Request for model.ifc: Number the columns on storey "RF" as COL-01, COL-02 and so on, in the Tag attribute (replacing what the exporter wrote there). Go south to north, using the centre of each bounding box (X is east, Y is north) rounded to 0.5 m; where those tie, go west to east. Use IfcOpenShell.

First a look at what the model holds.

```python
import ifcopenshell
import ifcopenshell.util.element
import ifcopenshell.util.placement

model = ifcopenshell.open("model.ifc")
print(model.schema)
storey = next(s for s in model.by_type("IfcBuildingStorey") if s.Name == "RF")
columns = [e for e in ifcopenshell.util.element.get_decomposition(storey) if e.is_a("IfcColumn")]
for e in sorted(columns, key=lambda e: e.id()):
    origin = ifcopenshell.util.placement.get_local_placement(e.ObjectPlacement)[:3, 3]
    print(e.id(), e.Tag, e.Name, origin.round(2) + 0.0, sep=" | ")
```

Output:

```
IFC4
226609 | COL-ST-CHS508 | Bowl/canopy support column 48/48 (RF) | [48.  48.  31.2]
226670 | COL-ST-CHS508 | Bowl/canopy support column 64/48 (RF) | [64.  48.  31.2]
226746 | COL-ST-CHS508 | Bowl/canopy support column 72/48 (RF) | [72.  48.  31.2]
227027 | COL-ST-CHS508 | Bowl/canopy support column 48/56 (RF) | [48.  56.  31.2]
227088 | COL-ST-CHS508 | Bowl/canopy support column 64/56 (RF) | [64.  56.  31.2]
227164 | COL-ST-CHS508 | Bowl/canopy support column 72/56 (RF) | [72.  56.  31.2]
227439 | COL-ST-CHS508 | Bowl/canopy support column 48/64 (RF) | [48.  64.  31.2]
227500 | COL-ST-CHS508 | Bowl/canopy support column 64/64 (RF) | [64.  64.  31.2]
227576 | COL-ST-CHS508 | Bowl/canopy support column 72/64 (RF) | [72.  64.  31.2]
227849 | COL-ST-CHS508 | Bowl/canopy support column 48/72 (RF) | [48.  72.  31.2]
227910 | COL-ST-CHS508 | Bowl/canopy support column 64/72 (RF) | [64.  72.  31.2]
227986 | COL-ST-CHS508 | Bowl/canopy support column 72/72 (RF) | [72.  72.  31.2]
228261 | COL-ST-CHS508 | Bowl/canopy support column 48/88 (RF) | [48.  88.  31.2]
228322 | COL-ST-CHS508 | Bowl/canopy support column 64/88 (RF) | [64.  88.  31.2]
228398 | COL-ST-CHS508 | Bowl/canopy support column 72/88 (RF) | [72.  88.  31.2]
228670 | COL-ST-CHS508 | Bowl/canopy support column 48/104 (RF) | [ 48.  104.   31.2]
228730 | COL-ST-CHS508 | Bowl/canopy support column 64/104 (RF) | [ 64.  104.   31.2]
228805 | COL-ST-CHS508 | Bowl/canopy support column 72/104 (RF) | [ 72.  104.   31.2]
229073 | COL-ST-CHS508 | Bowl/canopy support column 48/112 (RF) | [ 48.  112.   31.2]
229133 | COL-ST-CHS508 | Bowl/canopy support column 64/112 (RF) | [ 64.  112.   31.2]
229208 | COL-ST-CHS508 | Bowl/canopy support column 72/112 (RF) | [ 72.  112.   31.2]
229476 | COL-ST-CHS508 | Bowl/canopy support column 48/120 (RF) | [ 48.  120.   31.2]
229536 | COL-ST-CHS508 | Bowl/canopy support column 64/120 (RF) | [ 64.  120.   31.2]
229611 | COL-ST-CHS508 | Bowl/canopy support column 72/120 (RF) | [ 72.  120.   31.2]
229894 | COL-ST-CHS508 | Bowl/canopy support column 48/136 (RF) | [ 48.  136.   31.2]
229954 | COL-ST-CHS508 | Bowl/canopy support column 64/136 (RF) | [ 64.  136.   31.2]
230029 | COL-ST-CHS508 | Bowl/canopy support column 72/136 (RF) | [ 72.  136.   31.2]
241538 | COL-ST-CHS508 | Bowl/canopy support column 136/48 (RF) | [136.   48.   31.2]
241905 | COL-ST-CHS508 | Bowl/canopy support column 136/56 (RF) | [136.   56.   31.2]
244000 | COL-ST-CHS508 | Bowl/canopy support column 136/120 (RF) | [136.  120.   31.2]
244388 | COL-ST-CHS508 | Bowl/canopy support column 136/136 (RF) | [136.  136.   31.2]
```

```python
import ifcopenshell
import ifcopenshell.geom
import ifcopenshell.util.element
import ifcopenshell.util.shape

model = ifcopenshell.open("model.ifc")
settings = ifcopenshell.geom.settings()
settings.set("use-world-coords", True)


def centre(element):
    shape = ifcopenshell.geom.create_shape(settings, element)
    return ifcopenshell.util.shape.get_bbox_centroid(shape.geometry)


storey = next(s for s in model.by_type("IfcBuildingStorey") if s.Name == "RF")
columns = [e for e in ifcopenshell.util.element.get_decomposition(storey) if e.is_a("IfcColumn")]

# Insertion points can sit at a corner or the storey origin, so sort by the geometry (in metres).
centres = {e: centre(e) for e in columns}
columns.sort(key=lambda e: (round(centres[e][1] / 0.5), centres[e][0]))

for i, e in enumerate(columns, start=1):
    number = f"COL-{i:02d}"
    e.Tag = number
    print(e.id(), number)

model.write("model-out.ifc")
```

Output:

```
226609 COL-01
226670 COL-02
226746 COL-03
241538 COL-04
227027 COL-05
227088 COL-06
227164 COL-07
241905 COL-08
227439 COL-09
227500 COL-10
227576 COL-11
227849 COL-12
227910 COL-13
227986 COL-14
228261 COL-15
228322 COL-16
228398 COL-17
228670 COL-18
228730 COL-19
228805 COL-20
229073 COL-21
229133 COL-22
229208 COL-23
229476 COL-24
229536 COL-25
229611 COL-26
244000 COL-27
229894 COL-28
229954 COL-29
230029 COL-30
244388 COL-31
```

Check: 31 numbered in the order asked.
